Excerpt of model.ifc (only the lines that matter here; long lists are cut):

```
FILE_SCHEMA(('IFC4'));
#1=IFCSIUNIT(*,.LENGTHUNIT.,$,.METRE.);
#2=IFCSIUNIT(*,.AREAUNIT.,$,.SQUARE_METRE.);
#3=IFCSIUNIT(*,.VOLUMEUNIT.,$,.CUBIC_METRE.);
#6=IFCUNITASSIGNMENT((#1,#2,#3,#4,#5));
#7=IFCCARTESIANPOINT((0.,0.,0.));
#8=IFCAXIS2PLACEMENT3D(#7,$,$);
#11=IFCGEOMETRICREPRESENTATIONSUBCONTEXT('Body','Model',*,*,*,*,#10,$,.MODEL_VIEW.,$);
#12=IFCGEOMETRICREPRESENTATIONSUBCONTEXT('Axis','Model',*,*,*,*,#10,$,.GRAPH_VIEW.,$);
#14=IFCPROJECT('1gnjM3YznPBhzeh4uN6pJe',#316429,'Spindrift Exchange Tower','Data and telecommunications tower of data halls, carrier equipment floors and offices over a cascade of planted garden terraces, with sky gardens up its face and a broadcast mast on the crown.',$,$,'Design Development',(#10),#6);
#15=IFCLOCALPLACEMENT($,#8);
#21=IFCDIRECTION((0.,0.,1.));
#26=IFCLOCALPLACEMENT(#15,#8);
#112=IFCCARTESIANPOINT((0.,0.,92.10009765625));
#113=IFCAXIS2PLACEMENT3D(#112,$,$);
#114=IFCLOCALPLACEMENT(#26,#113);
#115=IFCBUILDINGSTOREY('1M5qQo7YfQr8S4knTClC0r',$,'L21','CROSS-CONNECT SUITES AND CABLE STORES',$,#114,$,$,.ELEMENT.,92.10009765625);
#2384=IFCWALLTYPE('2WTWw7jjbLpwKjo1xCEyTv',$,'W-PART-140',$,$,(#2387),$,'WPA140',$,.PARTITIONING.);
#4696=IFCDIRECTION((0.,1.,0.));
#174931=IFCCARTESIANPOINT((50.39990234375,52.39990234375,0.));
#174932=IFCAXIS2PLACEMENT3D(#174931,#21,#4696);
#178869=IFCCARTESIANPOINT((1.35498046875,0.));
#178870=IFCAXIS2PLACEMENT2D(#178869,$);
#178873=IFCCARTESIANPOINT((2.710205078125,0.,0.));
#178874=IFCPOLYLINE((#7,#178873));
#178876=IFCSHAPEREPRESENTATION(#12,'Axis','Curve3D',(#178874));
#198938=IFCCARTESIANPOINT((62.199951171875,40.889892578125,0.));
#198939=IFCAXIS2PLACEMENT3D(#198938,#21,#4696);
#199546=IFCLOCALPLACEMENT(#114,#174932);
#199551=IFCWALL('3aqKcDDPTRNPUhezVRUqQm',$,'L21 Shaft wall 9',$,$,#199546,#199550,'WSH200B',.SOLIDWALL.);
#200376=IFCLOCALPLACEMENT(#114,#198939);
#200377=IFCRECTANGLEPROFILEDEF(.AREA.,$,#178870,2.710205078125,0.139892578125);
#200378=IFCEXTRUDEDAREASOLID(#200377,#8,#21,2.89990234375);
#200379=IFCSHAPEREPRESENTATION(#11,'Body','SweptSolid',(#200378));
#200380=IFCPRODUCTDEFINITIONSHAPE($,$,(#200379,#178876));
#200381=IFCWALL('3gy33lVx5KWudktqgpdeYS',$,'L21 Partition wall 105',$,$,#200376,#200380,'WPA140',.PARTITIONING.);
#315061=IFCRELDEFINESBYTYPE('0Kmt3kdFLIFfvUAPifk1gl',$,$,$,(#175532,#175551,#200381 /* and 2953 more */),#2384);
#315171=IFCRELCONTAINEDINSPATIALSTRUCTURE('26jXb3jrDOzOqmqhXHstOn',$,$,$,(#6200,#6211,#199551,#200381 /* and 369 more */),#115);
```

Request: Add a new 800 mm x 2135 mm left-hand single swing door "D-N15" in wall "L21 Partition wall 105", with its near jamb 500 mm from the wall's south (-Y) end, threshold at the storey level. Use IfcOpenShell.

```python
import numpy as np
import ifcopenshell
import ifcopenshell.api.feature
import ifcopenshell.api.geometry
import ifcopenshell.api.root
import ifcopenshell.api.spatial
import ifcopenshell.geom
import ifcopenshell.util.element
import ifcopenshell.util.placement
import ifcopenshell.util.representation
import ifcopenshell.util.shape
import ifcopenshell.util.unit

model = ifcopenshell.open("model.ifc")
unit_scale = ifcopenshell.util.unit.calculate_unit_scale(model)
settings = ifcopenshell.geom.settings()


def volume(element):
    """Net volume in cubic metres, openings subtracted."""
    shape = ifcopenshell.geom.create_shape(settings, element)
    return ifcopenshell.util.shape.get_volume(shape.geometry)


wall = model.by_guid("3gy33lVx5KWudktqgpdeYS")
storey = ifcopenshell.util.element.get_container(wall, ifc_class="IfcBuildingStorey")
context = ifcopenshell.util.representation.get_context(model, "Model", "Body", "MODEL_VIEW")
before = volume(wall)

width, height, from_end, sill = 0.8, 2.135, 0.5, 0.0  # metres

# The wall runs along its own X axis, and the end named is its -X end.
wall_shape = ifcopenshell.geom.create_shape(settings, wall)
x, y, z = ifcopenshell.util.shape.get_vertices(wall_shape.geometry).T
start = x.min() + from_end
face, thickness = float(y.min()), float(y.max() - y.min())
wall_matrix = ifcopenshell.util.placement.get_local_placement(wall.ObjectPlacement)
level = ifcopenshell.util.placement.get_local_placement(storey.ObjectPlacement)[2, 3]


def in_wall(x, y):
    """Placement at x, y metres in the wall's axes, at sill height."""
    matrix = wall_matrix.copy()
    matrix[:, 3] = wall_matrix @ np.array([x / unit_scale, y / unit_scale, 0.0, 1.0])
    matrix[2, 3] = level + sill / unit_scale
    return matrix


# Opening: a box that overshoots both wall faces by 50 mm.
opening = ifcopenshell.api.root.create_entity(model, ifc_class="IfcOpeningElement", predefined_type="OPENING")
box = ifcopenshell.api.geometry.add_wall_representation(
    model, context=context, length=width, height=height, thickness=thickness + 0.1
)
ifcopenshell.api.geometry.assign_representation(model, product=opening, representation=box)
ifcopenshell.api.geometry.edit_object_placement(model, product=opening, matrix=in_wall(start, face - 0.05), is_si=False)
ifcopenshell.api.feature.add_feature(model, feature=opening, element=wall)

door = ifcopenshell.api.root.create_entity(model, ifc_class="IfcDoor", name="D-N15", predefined_type="DOOR")
door.OverallWidth, door.OverallHeight = width / unit_scale, height / unit_scale
door.OperationType = "SINGLE_SWING_LEFT"
body = ifcopenshell.api.geometry.add_door_representation(
    model,
    context=context,
    overall_width=door.OverallWidth,
    overall_height=door.OverallHeight,
    operation_type="SINGLE_SWING_LEFT",
    lining_properties={"LiningDepth": thickness / unit_scale, "ThresholdDepth": thickness / unit_scale},
)
ifcopenshell.api.geometry.assign_representation(model, product=door, representation=body)
ifcopenshell.api.spatial.assign_container(model, products=[door], relating_structure=storey)
ifcopenshell.api.feature.add_filling(model, opening=opening, element=door)

# The lining spans the wall, so the door starts at the wall face.
ifcopenshell.api.geometry.edit_object_placement(model, product=door, matrix=in_wall(start, face), is_si=False)

after = volume(wall)

print(f"wall volume {before:.3f} -> {after:.3f} m3")

model.write("model_updated.ifc")
```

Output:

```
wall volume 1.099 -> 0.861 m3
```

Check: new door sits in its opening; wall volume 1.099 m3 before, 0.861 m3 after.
